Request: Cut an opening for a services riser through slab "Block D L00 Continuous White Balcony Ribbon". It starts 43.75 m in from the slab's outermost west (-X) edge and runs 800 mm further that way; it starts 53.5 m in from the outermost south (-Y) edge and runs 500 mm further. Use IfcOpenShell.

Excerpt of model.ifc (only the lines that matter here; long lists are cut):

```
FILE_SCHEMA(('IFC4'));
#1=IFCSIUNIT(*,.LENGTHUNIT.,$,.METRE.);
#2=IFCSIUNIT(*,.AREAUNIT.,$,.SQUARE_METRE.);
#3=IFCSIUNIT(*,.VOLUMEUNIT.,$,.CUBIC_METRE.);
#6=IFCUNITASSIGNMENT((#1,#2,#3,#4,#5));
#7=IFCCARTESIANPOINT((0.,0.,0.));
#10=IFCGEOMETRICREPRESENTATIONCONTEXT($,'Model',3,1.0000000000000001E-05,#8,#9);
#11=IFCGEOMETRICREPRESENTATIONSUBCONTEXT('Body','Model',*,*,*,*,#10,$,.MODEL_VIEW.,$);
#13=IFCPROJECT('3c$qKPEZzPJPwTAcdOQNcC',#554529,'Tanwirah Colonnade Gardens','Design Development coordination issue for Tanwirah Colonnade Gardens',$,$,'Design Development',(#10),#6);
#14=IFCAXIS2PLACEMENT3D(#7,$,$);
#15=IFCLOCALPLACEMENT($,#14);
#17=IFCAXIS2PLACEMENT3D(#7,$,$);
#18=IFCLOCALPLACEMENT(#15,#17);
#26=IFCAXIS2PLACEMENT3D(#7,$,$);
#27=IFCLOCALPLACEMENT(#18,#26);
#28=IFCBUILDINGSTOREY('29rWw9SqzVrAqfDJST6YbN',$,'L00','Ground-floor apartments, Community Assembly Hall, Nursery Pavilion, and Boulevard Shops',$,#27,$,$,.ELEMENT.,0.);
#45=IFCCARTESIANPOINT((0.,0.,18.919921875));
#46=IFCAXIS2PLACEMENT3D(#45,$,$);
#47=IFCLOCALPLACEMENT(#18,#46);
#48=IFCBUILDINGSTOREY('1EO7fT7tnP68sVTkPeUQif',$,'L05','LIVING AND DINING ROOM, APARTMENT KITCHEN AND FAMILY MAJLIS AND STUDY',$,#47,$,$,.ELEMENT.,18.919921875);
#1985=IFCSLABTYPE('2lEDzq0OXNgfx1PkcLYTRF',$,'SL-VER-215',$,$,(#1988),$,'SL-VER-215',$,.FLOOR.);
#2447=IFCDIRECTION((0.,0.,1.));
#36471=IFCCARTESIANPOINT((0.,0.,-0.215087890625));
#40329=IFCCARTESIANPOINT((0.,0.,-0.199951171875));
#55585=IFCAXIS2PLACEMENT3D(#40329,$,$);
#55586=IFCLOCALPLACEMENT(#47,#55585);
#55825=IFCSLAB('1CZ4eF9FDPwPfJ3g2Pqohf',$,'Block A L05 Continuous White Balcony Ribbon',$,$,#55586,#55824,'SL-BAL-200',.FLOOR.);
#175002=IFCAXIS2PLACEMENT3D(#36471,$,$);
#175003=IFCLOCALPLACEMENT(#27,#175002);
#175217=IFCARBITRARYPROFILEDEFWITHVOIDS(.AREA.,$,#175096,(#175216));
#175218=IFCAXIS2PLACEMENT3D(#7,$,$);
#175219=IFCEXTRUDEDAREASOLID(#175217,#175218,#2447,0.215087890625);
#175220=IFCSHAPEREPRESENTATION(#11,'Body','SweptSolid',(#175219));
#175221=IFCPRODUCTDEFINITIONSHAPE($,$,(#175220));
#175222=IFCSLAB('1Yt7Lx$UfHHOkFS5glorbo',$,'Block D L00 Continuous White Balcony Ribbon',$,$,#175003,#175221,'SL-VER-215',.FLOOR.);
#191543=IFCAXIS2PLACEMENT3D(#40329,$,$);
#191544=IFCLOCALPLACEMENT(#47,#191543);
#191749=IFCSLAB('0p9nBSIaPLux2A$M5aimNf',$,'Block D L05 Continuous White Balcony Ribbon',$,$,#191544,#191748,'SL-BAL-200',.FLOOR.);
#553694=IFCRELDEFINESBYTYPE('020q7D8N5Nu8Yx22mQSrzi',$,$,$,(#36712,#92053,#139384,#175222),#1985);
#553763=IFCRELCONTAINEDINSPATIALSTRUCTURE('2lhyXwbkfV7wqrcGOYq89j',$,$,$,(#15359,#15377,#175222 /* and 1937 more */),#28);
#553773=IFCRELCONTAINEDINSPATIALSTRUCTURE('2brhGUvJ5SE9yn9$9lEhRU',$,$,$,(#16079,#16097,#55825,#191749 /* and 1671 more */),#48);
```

```python
import numpy as np
import ifcopenshell
import ifcopenshell.api.feature
import ifcopenshell.api.geometry
import ifcopenshell.api.root
import ifcopenshell.geom
import ifcopenshell.util.placement
import ifcopenshell.util.representation
import ifcopenshell.util.shape
import ifcopenshell.util.unit

model = ifcopenshell.open("model.ifc")
unit_scale = ifcopenshell.util.unit.calculate_unit_scale(model)
settings = ifcopenshell.geom.settings()


def volume(element):
    """Net volume in cubic metres, openings subtracted."""
    shape = ifcopenshell.geom.create_shape(settings, element)
    return ifcopenshell.util.shape.get_volume(shape.geometry)


slab = model.by_guid("1Yt7Lx$UfHHOkFS5glorbo")
before = volume(slab)

# Extent in the slab's own axes, in metres. The edges named are its -X and -Y sides.
slab_shape = ifcopenshell.geom.create_shape(settings, slab)
vertices = ifcopenshell.util.shape.get_vertices(slab_shape.geometry)
x_min, y_min, bottom = vertices.min(axis=0)
top = vertices[:, 2].max()

opening = ifcopenshell.api.root.create_entity(model, ifc_class="IfcOpeningElement", name="Services riser opening", predefined_type="OPENING")
context = ifcopenshell.util.representation.get_context(model, "Model", "Body", "MODEL_VIEW")
width, depth = 0.8, 0.5
outline = [(0.0, 0.0), (width, 0.0), (width, depth), (0.0, depth), (0.0, 0.0)]
# Overshoot both faces by 50 mm so the cut is clean.
shape = ifcopenshell.api.geometry.add_slab_representation(
    model, context=context, depth=top - bottom + 0.1, polyline=outline
)
ifcopenshell.api.geometry.assign_representation(model, product=opening, representation=shape)

matrix = ifcopenshell.util.placement.get_local_placement(slab.ObjectPlacement)
matrix[:, 3] = matrix @ np.append(np.array([x_min + 43.75, y_min + 53.5, bottom - 0.05]) / unit_scale, 1.0)
ifcopenshell.api.geometry.edit_object_placement(model, product=opening, matrix=matrix, is_si=False)
ifcopenshell.api.feature.add_feature(model, feature=opening, element=slab)

after = volume(slab)

print(f"slab volume {before:.3f} -> {after:.3f} m3")

model.write("model_edited.ifc")
```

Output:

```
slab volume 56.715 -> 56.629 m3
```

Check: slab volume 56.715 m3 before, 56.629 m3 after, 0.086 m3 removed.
